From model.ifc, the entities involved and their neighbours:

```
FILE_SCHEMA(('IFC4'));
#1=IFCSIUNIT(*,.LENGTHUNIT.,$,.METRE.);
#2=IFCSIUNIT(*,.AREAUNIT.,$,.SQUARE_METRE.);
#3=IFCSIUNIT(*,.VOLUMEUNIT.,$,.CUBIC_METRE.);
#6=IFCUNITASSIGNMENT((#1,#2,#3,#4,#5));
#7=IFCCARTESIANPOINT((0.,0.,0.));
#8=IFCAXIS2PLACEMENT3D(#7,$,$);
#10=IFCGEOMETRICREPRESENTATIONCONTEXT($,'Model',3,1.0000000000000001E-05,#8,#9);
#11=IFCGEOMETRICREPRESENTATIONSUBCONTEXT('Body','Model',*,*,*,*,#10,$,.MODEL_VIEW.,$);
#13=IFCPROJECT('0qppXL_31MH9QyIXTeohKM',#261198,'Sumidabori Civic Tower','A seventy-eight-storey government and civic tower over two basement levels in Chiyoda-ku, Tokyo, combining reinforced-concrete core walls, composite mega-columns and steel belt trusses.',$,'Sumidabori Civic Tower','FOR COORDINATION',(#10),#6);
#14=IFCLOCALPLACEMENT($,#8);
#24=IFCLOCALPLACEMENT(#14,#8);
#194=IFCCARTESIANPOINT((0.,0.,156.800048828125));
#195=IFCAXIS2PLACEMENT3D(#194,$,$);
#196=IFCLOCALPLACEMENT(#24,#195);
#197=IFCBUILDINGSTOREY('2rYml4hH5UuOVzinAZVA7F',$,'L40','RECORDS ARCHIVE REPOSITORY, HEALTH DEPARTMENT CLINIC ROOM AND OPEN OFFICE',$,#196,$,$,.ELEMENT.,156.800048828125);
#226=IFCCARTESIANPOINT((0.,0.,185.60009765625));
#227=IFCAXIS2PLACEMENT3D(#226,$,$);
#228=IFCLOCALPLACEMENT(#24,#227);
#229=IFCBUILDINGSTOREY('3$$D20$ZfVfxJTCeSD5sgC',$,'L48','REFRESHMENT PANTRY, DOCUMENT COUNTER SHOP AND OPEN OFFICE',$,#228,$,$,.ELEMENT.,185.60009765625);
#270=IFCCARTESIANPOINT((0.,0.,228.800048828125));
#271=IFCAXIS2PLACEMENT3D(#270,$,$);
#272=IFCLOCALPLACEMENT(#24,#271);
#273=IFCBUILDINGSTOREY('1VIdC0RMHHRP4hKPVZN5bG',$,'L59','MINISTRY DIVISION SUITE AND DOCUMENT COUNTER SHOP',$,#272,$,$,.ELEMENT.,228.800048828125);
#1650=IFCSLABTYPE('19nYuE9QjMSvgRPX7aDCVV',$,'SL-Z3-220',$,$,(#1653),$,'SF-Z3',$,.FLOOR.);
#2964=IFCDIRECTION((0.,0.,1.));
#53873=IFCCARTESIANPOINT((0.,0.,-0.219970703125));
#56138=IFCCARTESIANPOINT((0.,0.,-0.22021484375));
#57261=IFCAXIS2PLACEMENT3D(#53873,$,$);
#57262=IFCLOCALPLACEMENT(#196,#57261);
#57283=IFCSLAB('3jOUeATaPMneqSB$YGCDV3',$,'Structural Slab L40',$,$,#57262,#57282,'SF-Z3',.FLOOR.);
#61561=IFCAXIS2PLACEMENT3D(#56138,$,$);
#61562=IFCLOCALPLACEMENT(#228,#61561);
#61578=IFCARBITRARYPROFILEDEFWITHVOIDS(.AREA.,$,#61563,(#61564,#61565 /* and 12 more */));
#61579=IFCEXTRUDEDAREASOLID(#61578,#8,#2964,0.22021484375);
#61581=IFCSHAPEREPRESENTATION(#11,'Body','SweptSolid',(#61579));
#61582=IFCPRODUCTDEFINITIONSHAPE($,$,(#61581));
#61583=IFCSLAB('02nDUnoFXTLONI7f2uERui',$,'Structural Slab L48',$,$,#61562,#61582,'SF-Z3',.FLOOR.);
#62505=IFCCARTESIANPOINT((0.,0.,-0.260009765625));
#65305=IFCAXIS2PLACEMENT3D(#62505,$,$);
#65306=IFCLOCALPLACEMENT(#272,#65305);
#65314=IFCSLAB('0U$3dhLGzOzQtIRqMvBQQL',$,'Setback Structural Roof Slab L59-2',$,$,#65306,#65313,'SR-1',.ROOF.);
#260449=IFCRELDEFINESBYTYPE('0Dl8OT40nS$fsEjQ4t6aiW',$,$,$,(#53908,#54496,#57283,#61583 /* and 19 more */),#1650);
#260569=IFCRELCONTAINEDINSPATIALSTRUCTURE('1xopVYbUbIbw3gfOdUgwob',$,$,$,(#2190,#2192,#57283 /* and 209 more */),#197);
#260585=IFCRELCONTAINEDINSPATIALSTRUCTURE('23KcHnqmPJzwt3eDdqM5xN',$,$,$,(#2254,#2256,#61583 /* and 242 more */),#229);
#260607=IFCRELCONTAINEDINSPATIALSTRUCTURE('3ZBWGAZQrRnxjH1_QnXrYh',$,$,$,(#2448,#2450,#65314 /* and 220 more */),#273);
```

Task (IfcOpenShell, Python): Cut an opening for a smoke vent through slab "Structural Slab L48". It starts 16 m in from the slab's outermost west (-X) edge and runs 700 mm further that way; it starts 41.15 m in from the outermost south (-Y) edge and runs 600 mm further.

```python
import numpy as np
import ifcopenshell
import ifcopenshell.api.feature
import ifcopenshell.api.geometry
import ifcopenshell.api.root
import ifcopenshell.geom
import ifcopenshell.util.placement
import ifcopenshell.util.representation
import ifcopenshell.util.shape
import ifcopenshell.util.unit

model = ifcopenshell.open("model.ifc")
unit_scale = ifcopenshell.util.unit.calculate_unit_scale(model)
settings = ifcopenshell.geom.settings()


def volume(element):
    """Net volume in cubic metres, openings subtracted."""
    shape = ifcopenshell.geom.create_shape(settings, element)
    return ifcopenshell.util.shape.get_volume(shape.geometry)


slab = model.by_guid("02nDUnoFXTLONI7f2uERui")
before = volume(slab)

# Extent in the slab's own axes, in metres. The edges named are its -X and -Y sides.
slab_shape = ifcopenshell.geom.create_shape(settings, slab)
vertices = ifcopenshell.util.shape.get_vertices(slab_shape.geometry)
x_min, y_min, bottom = vertices.min(axis=0)
top = vertices[:, 2].max()

opening = ifcopenshell.api.root.create_entity(model, ifc_class="IfcOpeningElement", name="Smoke vent opening", predefined_type="OPENING")
context = ifcopenshell.util.representation.get_context(model, "Model", "Body", "MODEL_VIEW")
width, depth = 0.7, 0.6
outline = [(0.0, 0.0), (width, 0.0), (width, depth), (0.0, depth), (0.0, 0.0)]
# Overshoot both faces by 50 mm so the cut is clean.
shape = ifcopenshell.api.geometry.add_slab_representation(
    model, context=context, depth=top - bottom + 0.1, polyline=outline
)
ifcopenshell.api.geometry.assign_representation(model, product=opening, representation=shape)

matrix = ifcopenshell.util.placement.get_local_placement(slab.ObjectPlacement)
matrix[:, 3] = matrix @ np.append(np.array([x_min + 16, y_min + 41.15, bottom - 0.05]) / unit_scale, 1.0)
ifcopenshell.api.geometry.edit_object_placement(model, product=opening, matrix=matrix, is_si=False)
ifcopenshell.api.feature.add_feature(model, feature=opening, element=slab)

after = volume(slab)

print(f"slab volume {before:.3f} -> {after:.3f} m3")

model.write("model_edited.ifc")
```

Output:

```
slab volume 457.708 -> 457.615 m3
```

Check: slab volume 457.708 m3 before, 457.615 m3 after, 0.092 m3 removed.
